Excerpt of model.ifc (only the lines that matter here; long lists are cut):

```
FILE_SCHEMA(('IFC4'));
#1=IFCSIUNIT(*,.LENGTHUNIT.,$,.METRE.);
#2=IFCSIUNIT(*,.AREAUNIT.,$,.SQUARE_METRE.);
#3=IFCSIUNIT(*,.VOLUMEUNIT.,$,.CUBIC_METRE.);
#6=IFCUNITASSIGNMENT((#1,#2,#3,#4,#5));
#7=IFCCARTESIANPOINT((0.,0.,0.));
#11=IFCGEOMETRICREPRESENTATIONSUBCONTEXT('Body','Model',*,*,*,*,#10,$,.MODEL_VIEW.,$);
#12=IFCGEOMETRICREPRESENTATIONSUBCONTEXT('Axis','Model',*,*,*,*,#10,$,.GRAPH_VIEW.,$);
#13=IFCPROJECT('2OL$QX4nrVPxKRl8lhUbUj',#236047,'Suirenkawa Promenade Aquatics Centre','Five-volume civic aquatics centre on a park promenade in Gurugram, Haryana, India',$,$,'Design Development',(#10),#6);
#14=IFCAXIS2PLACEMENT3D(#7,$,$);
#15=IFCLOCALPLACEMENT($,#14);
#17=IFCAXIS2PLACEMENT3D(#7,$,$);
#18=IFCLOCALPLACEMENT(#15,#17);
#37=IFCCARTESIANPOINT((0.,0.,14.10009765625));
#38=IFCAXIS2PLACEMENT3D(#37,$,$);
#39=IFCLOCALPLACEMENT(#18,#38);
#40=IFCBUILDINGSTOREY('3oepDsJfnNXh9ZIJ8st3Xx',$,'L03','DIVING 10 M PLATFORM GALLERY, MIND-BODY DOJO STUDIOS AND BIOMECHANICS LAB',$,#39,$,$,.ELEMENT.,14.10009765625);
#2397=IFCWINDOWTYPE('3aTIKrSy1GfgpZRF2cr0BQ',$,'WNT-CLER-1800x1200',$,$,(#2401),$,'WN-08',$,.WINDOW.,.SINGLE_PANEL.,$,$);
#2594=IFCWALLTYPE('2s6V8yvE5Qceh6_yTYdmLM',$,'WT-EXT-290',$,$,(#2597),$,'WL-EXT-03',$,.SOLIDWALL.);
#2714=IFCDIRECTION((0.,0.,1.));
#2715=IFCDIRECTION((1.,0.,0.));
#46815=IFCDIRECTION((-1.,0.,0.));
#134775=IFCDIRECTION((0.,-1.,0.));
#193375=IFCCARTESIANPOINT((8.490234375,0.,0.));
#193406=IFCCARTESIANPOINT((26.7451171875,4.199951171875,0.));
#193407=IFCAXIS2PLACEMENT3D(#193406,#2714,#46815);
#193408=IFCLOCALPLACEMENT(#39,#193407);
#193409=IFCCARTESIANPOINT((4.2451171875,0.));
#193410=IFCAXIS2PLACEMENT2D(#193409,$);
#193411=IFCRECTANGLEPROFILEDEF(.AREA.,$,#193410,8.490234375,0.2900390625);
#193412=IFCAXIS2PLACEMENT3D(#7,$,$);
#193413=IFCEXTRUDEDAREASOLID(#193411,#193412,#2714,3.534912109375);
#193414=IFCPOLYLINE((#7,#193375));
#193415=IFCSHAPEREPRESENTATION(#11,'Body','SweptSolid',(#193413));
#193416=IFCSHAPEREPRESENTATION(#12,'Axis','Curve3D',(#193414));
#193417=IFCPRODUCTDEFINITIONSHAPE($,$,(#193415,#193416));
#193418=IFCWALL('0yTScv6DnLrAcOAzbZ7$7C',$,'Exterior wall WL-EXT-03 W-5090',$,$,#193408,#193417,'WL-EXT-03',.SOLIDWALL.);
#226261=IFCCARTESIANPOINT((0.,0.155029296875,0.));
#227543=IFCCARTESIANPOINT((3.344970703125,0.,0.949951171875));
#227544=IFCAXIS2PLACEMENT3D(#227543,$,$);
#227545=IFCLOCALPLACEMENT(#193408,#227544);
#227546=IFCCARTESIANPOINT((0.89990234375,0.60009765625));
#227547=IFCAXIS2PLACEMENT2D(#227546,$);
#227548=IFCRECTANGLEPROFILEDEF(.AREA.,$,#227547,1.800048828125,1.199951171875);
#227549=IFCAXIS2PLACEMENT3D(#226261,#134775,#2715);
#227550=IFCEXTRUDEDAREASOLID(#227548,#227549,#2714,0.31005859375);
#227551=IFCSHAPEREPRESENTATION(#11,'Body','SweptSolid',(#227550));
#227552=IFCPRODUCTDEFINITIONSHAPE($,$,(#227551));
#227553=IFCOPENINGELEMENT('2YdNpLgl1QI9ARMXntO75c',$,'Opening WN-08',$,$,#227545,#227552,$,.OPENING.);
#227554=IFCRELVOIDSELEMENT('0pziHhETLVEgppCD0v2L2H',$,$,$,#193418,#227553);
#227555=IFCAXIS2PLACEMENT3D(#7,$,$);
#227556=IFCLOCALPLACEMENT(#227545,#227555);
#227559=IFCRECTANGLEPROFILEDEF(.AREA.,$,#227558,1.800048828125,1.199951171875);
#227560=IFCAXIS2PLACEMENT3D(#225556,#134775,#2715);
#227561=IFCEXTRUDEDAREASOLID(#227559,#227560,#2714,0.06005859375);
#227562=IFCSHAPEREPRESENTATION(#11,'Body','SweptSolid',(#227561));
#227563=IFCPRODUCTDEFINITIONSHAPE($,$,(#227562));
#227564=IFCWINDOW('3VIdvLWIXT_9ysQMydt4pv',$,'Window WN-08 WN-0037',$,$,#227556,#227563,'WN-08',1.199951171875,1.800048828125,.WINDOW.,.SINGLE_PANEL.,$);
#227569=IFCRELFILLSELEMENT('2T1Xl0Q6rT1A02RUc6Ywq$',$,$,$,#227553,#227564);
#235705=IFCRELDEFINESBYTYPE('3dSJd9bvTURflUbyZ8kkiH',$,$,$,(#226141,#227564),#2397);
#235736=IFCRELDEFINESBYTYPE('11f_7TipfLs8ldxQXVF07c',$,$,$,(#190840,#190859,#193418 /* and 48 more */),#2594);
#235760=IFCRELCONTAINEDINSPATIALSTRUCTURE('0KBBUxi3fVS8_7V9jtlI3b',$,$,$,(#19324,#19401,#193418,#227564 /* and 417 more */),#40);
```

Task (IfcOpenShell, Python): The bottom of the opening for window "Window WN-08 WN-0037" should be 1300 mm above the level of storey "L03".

```python
import numpy as np
import ifcopenshell
import ifcopenshell.api.geometry
import ifcopenshell.geom
import ifcopenshell.util.element
import ifcopenshell.util.placement
import ifcopenshell.util.shape
import ifcopenshell.util.unit

model = ifcopenshell.open("model.ifc")
unit_scale = ifcopenshell.util.unit.calculate_unit_scale(model)

window = model.by_guid("3VIdvLWIXT_9ysQMydt4pv")
opening = window.FillsVoids[0].RelatingOpeningElement
storey = ifcopenshell.util.element.get_container(window, ifc_class="IfcBuildingStorey")
level = ifcopenshell.util.placement.get_local_placement(storey.ObjectPlacement)[2, 3]

# The opening's origin need not be at the sill, so measure its lowest point.
shape = ifcopenshell.geom.create_shape(ifcopenshell.geom.settings(), opening)
bottom = ifcopenshell.util.shape.get_shape_bottom_elevation(shape, shape.geometry) / unit_scale
dz = level + 1.3 - bottom

shift = np.array([0.0, 0.0, dz])
# The window is placed relative to its opening, so it follows when the opening moves.
matrix = ifcopenshell.util.placement.get_local_placement(opening.ObjectPlacement)
matrix[:3, 3] += shift
ifcopenshell.api.geometry.edit_object_placement(
    model, product=opening, matrix=matrix, is_si=False, should_transform_children=True
)

print(f"moved by {dz * unit_scale:+.3f} m")

model.write("model-out.ifc")
```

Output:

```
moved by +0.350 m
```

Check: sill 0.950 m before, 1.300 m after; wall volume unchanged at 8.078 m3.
